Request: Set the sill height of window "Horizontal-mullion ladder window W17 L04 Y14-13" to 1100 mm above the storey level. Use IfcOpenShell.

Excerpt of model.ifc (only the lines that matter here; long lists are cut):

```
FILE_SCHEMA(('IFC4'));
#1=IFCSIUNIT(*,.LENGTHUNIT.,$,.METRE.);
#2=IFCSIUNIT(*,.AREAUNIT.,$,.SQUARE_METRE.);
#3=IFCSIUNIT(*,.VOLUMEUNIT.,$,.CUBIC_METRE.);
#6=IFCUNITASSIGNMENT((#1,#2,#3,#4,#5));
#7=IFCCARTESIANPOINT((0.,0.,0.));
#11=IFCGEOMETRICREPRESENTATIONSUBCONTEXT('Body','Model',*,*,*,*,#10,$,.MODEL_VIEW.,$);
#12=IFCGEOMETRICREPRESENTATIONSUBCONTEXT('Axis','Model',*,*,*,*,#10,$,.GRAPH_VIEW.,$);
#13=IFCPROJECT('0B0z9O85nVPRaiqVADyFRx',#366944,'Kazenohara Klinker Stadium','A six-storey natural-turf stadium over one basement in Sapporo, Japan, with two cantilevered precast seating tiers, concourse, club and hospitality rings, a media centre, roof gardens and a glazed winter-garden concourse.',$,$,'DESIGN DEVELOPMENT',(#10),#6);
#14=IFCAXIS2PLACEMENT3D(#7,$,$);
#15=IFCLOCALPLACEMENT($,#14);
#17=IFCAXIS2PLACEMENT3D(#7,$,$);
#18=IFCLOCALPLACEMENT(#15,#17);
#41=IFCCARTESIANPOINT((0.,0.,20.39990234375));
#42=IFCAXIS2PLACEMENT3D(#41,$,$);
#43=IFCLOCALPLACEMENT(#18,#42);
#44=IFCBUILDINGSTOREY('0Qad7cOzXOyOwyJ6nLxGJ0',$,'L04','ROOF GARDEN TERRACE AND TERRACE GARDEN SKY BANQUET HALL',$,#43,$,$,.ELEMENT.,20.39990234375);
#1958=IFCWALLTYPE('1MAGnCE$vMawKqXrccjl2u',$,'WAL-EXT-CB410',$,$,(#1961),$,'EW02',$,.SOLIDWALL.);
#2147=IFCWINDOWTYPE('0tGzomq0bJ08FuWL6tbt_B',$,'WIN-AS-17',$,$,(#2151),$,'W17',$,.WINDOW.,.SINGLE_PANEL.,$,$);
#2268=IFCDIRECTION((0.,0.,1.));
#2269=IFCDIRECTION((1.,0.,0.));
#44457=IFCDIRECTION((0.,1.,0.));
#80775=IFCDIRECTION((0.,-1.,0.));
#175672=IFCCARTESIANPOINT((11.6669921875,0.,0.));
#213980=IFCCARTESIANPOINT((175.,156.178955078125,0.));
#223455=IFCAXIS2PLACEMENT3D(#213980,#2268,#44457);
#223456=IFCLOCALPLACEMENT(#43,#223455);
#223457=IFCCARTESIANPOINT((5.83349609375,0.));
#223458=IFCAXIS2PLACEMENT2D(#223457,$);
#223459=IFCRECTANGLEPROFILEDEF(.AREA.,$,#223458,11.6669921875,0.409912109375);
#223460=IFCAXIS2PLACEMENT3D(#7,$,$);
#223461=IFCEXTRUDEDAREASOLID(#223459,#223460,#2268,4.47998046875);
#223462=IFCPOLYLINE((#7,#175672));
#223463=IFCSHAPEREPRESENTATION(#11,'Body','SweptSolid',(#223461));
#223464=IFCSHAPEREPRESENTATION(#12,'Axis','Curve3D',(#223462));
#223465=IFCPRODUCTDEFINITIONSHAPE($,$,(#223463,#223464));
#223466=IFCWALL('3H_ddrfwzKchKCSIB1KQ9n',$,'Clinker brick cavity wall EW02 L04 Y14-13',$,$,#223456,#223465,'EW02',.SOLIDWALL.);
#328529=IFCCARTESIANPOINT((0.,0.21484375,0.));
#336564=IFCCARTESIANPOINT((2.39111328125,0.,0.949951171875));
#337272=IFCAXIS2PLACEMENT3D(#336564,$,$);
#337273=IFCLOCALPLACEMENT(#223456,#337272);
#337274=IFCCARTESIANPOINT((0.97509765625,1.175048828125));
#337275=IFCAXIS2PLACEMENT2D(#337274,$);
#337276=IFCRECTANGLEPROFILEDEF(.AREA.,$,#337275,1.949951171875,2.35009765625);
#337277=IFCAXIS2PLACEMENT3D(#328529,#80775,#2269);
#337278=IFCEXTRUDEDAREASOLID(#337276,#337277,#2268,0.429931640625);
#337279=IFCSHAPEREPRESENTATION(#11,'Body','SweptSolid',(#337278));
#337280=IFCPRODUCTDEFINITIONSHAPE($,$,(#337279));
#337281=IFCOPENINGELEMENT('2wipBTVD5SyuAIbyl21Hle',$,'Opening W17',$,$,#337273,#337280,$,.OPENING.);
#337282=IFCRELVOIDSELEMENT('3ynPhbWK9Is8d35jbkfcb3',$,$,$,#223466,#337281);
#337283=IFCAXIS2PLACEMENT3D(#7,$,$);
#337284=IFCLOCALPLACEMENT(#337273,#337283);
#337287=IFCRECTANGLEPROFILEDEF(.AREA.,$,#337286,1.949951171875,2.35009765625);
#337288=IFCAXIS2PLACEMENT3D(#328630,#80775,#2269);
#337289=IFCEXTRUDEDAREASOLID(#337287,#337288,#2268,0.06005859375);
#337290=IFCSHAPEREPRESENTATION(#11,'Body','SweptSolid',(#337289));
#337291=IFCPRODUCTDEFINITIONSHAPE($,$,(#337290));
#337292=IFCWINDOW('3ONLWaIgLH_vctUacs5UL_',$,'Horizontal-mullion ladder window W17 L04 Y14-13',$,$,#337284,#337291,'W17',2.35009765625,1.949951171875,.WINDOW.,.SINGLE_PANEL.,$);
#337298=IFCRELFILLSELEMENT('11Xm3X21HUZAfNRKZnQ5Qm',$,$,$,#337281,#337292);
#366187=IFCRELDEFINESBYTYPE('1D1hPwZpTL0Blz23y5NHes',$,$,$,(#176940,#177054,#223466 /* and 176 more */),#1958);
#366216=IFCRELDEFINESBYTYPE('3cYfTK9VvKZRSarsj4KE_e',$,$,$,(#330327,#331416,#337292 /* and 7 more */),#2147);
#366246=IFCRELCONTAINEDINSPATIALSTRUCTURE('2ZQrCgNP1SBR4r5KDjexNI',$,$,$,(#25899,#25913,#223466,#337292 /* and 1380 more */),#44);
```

```python
import numpy as np
import ifcopenshell
import ifcopenshell.api.geometry
import ifcopenshell.geom
import ifcopenshell.util.element
import ifcopenshell.util.placement
import ifcopenshell.util.shape
import ifcopenshell.util.unit

model = ifcopenshell.open("model.ifc")
unit_scale = ifcopenshell.util.unit.calculate_unit_scale(model)

window = model.by_guid("3ONLWaIgLH_vctUacs5UL_")
opening = window.FillsVoids[0].RelatingOpeningElement
storey = ifcopenshell.util.element.get_container(window, ifc_class="IfcBuildingStorey")
level = ifcopenshell.util.placement.get_local_placement(storey.ObjectPlacement)[2, 3]

# The opening's origin need not be at the sill, so measure its lowest point.
shape = ifcopenshell.geom.create_shape(ifcopenshell.geom.settings(), opening)
bottom = ifcopenshell.util.shape.get_shape_bottom_elevation(shape, shape.geometry) / unit_scale
dz = level + 1.1 / unit_scale - bottom

shift = np.array([0.0, 0.0, dz])
# The window is placed relative to its opening, so it follows when the opening moves.
matrix = ifcopenshell.util.placement.get_local_placement(opening.ObjectPlacement)
matrix[:3, 3] += shift
ifcopenshell.api.geometry.edit_object_placement(
    model, product=opening, matrix=matrix, is_si=False, should_transform_children=True
)

print(f"moved by {dz * unit_scale:+.3f} m")

model.write("model_v2.ifc")
```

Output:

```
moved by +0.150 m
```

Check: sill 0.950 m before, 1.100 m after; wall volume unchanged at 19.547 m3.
